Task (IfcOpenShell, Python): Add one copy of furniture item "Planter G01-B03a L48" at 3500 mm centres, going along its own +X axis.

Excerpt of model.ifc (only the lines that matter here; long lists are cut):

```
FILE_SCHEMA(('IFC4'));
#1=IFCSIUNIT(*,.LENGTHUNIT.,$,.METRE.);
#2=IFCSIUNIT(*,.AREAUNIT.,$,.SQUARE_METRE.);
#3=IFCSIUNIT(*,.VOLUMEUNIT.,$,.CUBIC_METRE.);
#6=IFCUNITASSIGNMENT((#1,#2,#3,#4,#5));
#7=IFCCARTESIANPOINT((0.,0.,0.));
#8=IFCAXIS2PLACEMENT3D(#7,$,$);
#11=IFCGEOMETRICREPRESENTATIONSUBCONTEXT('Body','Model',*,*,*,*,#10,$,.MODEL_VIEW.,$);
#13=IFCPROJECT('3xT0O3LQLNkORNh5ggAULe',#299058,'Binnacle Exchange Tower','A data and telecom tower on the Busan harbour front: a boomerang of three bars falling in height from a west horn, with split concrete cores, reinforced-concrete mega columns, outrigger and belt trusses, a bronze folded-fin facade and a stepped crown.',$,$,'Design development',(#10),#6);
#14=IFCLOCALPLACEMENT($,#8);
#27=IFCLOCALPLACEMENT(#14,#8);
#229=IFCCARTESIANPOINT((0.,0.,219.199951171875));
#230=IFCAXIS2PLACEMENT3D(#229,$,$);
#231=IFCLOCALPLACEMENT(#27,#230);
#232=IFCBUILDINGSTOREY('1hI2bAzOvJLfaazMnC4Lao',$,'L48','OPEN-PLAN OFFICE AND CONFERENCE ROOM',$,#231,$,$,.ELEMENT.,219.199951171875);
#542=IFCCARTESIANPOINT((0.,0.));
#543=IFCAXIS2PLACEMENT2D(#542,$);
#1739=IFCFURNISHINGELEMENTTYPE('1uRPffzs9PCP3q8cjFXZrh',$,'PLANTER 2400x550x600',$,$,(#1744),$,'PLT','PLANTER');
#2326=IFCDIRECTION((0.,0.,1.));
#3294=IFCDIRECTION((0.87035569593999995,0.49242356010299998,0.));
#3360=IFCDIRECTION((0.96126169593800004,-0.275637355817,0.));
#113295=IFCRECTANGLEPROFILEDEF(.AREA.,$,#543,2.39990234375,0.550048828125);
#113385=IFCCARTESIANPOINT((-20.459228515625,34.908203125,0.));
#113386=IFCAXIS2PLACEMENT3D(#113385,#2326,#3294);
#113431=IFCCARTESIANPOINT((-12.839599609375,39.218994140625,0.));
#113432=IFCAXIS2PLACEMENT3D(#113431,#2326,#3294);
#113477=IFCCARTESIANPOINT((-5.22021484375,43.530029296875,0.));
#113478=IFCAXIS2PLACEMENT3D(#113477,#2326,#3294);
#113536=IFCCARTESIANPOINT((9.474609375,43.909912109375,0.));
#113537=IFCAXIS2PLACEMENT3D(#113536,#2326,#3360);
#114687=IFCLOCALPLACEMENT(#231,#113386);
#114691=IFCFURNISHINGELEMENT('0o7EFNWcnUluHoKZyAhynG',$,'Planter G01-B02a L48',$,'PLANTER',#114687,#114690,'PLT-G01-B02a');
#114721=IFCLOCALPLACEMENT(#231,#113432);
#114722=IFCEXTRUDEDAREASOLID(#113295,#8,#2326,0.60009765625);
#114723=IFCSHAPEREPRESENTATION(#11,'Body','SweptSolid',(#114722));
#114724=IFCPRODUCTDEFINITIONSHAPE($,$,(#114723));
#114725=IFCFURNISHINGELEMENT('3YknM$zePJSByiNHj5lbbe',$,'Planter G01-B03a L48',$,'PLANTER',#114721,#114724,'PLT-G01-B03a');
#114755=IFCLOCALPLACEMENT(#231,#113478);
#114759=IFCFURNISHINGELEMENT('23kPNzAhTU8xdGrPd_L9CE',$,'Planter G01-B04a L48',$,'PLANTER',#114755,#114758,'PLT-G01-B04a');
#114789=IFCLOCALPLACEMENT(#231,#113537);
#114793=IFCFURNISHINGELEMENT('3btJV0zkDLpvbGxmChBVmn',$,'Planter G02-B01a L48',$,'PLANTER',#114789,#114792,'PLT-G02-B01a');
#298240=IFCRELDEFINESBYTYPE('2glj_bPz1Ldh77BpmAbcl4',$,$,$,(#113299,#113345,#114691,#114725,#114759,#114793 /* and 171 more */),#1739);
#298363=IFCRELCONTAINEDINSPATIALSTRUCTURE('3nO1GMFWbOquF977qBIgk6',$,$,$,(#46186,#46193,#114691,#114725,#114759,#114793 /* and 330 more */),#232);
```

```python
import ifcopenshell
import ifcopenshell.api.geometry
import ifcopenshell.api.root
import ifcopenshell.util.element
import ifcopenshell.util.placement
import ifcopenshell.util.unit

model = ifcopenshell.open("model.ifc")
unit_scale = ifcopenshell.util.unit.calculate_unit_scale(model)

source = model.by_guid("3YknM$zePJSByiNHj5lbbe")
base = ifcopenshell.util.placement.get_local_placement(source.ObjectPlacement)
step = base[:3, 0] * 3.5 / unit_scale

for i in range(1, 2):
    copy = ifcopenshell.api.root.copy_class(model, product=source)
    copy.Representation = ifcopenshell.util.element.copy_deep(
        model, source.Representation, exclude=["IfcGeometricRepresentationContext", "IfcRepresentationMap"]
    )
    copy.Tag = None
    matrix = base.copy()
    matrix[:3, 3] += i * step
    print("added at", matrix[:3, 3].round(3) + 0.0)
    ifcopenshell.api.geometry.edit_object_placement(model, product=copy, matrix=matrix, is_si=False)

model.write("model_edited.ifc")
```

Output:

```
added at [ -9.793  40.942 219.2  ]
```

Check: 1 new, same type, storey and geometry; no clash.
